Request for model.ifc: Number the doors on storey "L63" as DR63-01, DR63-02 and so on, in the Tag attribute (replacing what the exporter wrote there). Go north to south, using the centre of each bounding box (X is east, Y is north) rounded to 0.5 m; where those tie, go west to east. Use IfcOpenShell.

First a look at what the model holds.

```python
import ifcopenshell
import ifcopenshell.util.element
import ifcopenshell.util.placement

model = ifcopenshell.open("model.ifc")
print(model.schema)
storey = next(s for s in model.by_type("IfcBuildingStorey") if s.Name == "L63")
doors = [e for e in ifcopenshell.util.element.get_decomposition(storey) if e.is_a("IfcDoor")]
for e in sorted(doors, key=lambda e: e.id()):
    origin = ifcopenshell.util.placement.get_local_placement(e.ObjectPlacement)[:3, 3]
    print(e.id(), e.Tag, e.Name, origin.round(2) + 0.0, sep=" | ")
```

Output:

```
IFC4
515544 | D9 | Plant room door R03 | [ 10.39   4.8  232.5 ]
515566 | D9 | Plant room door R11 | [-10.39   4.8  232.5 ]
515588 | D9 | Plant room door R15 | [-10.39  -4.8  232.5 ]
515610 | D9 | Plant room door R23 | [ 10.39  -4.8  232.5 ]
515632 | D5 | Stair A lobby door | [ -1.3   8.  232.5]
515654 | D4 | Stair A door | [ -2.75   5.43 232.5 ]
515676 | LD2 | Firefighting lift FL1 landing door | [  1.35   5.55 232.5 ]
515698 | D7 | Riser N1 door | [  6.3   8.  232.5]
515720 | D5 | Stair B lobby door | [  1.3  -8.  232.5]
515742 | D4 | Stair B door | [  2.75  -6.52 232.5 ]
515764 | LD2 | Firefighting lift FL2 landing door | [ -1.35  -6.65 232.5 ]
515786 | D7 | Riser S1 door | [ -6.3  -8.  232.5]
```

```python
import ifcopenshell
import ifcopenshell.geom
import ifcopenshell.util.element
import ifcopenshell.util.shape

model = ifcopenshell.open("model.ifc")
settings = ifcopenshell.geom.settings()
settings.set("use-world-coords", True)


def centre(element):
    shape = ifcopenshell.geom.create_shape(settings, element)
    return ifcopenshell.util.shape.get_bbox_centroid(shape.geometry)


storey = next(s for s in model.by_type("IfcBuildingStorey") if s.Name == "L63")
doors = [e for e in ifcopenshell.util.element.get_decomposition(storey) if e.is_a("IfcDoor")]

# Insertion points can sit at a corner or the storey origin, so sort by the geometry (in metres).
centres = {e: centre(e) for e in doors}
doors.sort(key=lambda e: (-round(centres[e][1] / 0.5), centres[e][0]))

for i, e in enumerate(doors, start=1):
    number = f"DR63-{i:02d}"
    e.Tag = number
    print(e.id(), number)

model.write("model_updated.ifc")
```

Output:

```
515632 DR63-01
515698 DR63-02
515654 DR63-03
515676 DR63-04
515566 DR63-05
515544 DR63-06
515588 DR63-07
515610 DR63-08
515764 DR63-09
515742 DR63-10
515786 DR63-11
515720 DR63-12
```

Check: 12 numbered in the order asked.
